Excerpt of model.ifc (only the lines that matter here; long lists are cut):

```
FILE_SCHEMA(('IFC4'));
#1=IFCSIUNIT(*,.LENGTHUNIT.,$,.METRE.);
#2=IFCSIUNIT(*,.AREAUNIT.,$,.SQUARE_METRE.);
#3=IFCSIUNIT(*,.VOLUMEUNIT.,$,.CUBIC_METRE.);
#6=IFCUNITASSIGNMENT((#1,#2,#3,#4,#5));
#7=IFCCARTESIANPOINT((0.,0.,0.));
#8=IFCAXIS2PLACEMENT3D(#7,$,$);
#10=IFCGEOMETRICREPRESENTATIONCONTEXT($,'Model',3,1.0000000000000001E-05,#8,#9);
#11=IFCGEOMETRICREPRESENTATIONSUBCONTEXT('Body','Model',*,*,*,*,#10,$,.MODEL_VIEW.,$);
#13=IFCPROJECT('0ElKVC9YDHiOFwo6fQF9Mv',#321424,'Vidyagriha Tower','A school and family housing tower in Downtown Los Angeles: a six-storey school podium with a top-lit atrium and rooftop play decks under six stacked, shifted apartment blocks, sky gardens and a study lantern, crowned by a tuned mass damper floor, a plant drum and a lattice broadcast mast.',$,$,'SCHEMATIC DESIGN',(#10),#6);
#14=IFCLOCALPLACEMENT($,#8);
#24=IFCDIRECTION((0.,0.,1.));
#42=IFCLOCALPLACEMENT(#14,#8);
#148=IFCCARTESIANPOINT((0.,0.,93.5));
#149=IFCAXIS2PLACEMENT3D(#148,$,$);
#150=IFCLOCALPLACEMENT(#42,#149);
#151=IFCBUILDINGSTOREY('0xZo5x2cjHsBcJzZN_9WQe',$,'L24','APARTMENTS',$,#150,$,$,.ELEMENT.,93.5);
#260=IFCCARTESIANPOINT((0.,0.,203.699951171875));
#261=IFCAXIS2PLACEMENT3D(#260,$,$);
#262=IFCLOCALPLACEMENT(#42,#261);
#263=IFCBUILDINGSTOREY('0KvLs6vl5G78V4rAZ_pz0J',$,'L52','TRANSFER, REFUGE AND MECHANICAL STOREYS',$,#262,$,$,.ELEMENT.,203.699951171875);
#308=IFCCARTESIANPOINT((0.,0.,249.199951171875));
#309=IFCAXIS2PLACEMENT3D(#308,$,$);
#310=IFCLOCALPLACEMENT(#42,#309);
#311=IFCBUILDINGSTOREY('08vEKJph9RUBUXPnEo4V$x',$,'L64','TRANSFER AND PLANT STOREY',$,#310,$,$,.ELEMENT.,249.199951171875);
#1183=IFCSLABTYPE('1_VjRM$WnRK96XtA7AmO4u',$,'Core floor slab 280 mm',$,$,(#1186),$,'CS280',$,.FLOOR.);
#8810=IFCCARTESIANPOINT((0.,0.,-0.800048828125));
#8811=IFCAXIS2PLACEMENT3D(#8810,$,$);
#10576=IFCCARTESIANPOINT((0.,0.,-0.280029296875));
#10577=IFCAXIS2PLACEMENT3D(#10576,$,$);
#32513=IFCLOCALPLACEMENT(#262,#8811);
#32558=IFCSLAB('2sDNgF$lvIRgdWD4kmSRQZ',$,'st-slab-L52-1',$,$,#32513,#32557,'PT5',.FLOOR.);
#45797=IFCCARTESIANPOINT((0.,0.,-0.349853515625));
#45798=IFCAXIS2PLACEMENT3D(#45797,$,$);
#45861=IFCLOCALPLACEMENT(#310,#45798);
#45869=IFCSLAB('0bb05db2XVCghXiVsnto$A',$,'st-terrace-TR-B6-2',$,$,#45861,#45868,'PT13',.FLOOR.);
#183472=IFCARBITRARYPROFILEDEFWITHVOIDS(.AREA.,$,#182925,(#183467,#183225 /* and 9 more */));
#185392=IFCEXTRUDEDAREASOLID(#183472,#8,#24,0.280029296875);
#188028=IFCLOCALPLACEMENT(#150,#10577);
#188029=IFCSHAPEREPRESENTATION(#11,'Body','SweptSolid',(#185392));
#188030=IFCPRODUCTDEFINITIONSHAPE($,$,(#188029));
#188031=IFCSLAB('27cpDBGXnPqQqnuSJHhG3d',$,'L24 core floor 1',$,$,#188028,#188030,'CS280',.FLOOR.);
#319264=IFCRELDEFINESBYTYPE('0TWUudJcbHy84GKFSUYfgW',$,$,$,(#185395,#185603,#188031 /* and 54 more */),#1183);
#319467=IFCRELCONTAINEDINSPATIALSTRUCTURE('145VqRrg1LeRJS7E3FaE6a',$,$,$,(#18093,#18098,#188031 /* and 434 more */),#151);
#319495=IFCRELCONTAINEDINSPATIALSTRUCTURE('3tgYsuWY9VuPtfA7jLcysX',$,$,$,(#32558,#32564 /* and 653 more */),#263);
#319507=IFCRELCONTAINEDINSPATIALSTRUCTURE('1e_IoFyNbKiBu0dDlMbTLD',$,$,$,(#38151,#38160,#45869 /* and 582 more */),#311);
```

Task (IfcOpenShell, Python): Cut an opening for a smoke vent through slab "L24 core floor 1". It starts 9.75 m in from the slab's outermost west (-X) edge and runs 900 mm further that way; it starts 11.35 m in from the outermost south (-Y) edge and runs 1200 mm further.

```python
import numpy as np
import ifcopenshell
import ifcopenshell.api.feature
import ifcopenshell.api.geometry
import ifcopenshell.api.root
import ifcopenshell.geom
import ifcopenshell.util.placement
import ifcopenshell.util.representation
import ifcopenshell.util.shape
import ifcopenshell.util.unit

model = ifcopenshell.open("model.ifc")
unit_scale = ifcopenshell.util.unit.calculate_unit_scale(model)
settings = ifcopenshell.geom.settings()


def volume(element):
    """Net volume in cubic metres, openings subtracted."""
    shape = ifcopenshell.geom.create_shape(settings, element)
    return ifcopenshell.util.shape.get_volume(shape.geometry)


slab = model.by_guid("27cpDBGXnPqQqnuSJHhG3d")
before = volume(slab)

# Extent in the slab's own axes, in metres. The edges named are its -X and -Y sides.
slab_shape = ifcopenshell.geom.create_shape(settings, slab)
vertices = ifcopenshell.util.shape.get_vertices(slab_shape.geometry)
x_min, y_min, bottom = vertices.min(axis=0)
top = vertices[:, 2].max()

opening = ifcopenshell.api.root.create_entity(model, ifc_class="IfcOpeningElement", name="Smoke vent opening", predefined_type="OPENING")
context = ifcopenshell.util.representation.get_context(model, "Model", "Body", "MODEL_VIEW")
width, depth = 0.9, 1.2
outline = [(0.0, 0.0), (width, 0.0), (width, depth), (0.0, depth), (0.0, 0.0)]
# Overshoot both faces by 50 mm so the cut is clean.
shape = ifcopenshell.api.geometry.add_slab_representation(
    model, context=context, depth=top - bottom + 0.1, polyline=outline
)
ifcopenshell.api.geometry.assign_representation(model, product=opening, representation=shape)

matrix = ifcopenshell.util.placement.get_local_placement(slab.ObjectPlacement)
matrix[:, 3] = matrix @ np.append(np.array([x_min + 9.75, y_min + 11.35, bottom - 0.05]) / unit_scale, 1.0)
ifcopenshell.api.geometry.edit_object_placement(model, product=opening, matrix=matrix, is_si=False)
ifcopenshell.api.feature.add_feature(model, feature=opening, element=slab)

after = volume(slab)

print(f"slab volume {before:.3f} -> {after:.3f} m3")

model.write("model_rev.ifc")
```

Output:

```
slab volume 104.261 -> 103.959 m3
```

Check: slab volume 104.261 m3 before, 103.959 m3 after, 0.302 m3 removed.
